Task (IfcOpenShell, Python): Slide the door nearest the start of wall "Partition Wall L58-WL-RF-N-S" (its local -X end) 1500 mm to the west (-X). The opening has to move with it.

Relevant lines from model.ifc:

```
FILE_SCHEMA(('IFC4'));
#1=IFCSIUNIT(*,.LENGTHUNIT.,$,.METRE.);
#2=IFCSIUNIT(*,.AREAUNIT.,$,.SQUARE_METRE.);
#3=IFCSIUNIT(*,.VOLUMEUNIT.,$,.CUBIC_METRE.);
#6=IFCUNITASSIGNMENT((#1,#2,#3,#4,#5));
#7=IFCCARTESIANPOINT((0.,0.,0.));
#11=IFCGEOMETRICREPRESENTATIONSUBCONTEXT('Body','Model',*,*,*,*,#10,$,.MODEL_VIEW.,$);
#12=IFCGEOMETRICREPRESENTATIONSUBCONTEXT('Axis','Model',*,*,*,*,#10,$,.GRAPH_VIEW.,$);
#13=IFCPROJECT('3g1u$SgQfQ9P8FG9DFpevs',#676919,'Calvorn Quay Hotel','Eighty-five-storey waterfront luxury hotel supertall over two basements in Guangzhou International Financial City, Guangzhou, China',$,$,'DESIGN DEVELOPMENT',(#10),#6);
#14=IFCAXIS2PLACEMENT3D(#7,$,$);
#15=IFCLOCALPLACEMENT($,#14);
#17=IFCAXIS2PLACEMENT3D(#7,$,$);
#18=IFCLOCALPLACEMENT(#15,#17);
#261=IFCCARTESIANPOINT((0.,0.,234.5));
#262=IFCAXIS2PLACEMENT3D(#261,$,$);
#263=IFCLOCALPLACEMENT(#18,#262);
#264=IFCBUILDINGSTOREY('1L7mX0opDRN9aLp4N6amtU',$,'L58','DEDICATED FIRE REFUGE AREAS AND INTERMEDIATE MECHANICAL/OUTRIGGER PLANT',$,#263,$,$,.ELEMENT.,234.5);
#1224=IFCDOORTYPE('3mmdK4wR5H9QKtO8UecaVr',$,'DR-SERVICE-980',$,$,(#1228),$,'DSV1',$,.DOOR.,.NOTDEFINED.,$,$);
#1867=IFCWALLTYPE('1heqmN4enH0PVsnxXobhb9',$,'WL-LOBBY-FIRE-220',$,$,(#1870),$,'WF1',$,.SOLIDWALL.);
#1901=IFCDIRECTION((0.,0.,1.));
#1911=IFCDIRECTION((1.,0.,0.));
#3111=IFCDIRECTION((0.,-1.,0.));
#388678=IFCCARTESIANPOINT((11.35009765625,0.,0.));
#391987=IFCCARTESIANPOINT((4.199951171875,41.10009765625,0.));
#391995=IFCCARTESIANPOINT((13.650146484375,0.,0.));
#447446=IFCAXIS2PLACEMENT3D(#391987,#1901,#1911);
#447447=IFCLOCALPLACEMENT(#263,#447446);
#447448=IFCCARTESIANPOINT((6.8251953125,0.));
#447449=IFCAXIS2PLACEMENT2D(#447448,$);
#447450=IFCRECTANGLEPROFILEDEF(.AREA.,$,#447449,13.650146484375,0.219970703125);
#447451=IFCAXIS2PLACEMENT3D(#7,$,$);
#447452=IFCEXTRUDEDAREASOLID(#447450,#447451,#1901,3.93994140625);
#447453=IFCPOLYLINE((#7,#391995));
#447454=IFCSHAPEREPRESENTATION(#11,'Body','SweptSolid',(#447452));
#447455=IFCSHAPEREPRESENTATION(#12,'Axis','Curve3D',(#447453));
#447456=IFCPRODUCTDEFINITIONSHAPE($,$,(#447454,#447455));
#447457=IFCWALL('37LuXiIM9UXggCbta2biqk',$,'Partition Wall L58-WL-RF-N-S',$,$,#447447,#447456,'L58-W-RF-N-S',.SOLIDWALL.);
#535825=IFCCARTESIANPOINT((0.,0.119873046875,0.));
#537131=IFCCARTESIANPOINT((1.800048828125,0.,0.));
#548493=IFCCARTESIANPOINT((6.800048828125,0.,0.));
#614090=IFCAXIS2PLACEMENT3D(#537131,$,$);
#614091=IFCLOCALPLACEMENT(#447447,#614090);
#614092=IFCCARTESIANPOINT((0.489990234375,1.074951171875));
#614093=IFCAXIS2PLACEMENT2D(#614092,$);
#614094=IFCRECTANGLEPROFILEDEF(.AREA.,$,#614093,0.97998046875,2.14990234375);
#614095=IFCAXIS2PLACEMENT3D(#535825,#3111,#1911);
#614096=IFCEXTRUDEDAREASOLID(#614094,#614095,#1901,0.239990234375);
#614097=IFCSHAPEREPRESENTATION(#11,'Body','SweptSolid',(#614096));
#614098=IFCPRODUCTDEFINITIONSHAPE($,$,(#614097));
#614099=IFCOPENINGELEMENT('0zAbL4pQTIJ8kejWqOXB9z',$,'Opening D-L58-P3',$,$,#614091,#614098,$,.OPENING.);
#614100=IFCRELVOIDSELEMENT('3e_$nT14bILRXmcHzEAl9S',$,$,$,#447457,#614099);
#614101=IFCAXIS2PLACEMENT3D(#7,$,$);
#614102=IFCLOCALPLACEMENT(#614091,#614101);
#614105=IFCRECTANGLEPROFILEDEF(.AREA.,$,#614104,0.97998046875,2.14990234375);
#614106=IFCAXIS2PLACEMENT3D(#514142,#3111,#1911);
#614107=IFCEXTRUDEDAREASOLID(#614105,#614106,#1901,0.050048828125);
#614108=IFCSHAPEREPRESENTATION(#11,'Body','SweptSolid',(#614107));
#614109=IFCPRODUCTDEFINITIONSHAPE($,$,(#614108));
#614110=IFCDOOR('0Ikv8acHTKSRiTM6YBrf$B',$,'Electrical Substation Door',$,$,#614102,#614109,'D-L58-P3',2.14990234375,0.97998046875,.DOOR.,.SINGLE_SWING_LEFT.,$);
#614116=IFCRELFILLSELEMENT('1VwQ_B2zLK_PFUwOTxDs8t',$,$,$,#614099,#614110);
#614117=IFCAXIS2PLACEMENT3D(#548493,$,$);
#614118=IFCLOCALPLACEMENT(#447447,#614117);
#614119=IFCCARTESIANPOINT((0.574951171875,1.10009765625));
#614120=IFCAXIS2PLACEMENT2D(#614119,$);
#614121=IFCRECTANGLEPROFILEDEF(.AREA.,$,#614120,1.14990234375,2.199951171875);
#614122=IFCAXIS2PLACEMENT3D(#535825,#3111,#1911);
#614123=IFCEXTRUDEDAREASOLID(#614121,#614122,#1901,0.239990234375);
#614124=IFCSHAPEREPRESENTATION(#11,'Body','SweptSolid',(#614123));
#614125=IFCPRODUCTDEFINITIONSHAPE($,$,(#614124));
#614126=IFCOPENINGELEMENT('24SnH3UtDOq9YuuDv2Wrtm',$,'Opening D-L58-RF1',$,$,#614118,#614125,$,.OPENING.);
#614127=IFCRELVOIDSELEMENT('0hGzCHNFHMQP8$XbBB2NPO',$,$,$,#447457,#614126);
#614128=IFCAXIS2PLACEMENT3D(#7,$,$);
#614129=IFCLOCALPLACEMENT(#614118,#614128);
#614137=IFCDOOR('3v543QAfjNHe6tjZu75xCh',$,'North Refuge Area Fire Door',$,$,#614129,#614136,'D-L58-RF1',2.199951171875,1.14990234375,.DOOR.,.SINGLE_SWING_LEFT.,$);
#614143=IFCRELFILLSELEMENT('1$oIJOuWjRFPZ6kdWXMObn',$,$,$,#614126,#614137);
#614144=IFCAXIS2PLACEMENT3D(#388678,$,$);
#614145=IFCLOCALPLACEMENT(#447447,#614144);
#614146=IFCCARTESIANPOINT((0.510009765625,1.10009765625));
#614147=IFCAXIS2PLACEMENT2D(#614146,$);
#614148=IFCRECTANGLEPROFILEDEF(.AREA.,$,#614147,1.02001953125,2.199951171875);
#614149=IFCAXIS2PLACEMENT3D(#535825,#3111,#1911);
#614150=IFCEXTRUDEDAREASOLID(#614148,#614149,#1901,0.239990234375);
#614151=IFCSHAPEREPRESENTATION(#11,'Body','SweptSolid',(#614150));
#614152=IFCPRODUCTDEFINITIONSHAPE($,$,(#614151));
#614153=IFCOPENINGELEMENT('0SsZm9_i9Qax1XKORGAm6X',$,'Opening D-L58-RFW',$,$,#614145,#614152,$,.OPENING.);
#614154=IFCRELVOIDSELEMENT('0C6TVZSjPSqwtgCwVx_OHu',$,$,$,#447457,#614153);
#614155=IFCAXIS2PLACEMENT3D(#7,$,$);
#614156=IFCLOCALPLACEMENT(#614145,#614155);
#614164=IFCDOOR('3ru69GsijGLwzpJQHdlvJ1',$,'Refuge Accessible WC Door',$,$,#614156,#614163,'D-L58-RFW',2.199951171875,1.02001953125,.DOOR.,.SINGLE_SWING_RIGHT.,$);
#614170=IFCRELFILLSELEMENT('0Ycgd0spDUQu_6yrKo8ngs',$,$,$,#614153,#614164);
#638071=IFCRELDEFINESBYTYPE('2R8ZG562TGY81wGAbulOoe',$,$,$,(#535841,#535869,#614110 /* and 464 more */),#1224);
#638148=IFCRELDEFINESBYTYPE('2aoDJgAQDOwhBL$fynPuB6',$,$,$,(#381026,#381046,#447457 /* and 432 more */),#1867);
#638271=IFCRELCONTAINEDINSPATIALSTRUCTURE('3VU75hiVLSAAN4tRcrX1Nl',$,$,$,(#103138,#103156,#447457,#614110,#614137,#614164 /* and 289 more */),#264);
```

```python
import ifcopenshell
import ifcopenshell.api.geometry
import ifcopenshell.util.placement

model = ifcopenshell.open("model.ifc")

door = model.by_id(614110)
opening = door.FillsVoids[0].RelatingOpeningElement
wall = opening.VoidsElements[0].RelatingBuildingElement

wall_matrix = ifcopenshell.util.placement.get_local_placement(wall.ObjectPlacement)
shift = wall_matrix[:3, 0] * -1.5
before = ifcopenshell.util.placement.get_local_placement(door.ObjectPlacement)[:3, 3].copy()

# The door is placed relative to its opening, so it follows when the opening moves.
matrix = ifcopenshell.util.placement.get_local_placement(opening.ObjectPlacement)
matrix[:3, 3] += shift
ifcopenshell.api.geometry.edit_object_placement(
    model, product=opening, matrix=matrix, is_si=False, should_transform_children=True
)

after = ifcopenshell.util.placement.get_local_placement(door.ObjectPlacement)[:3, 3]
print("door moved by", (after - before).round(3) + 0.0)

model.write("model_rev.ifc")
```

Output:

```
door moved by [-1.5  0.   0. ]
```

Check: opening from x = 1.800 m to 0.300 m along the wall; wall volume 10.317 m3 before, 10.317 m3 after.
